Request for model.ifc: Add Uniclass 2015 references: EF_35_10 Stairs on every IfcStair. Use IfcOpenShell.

First a look at what the model holds.

```python
import ifcopenshell

model = ifcopenshell.open("model.ifc")
print(model.schema)
print("classifications:", [c.Name for c in model.by_type("IfcClassification")])
for ifc_class in ("IfcDoor", "IfcRoof", "IfcStair", "IfcWall", "IfcWindow"):
    print(ifc_class, len(model.by_type(ifc_class)))
```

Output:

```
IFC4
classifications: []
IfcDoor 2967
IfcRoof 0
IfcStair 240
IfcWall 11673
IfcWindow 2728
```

```python
import ifcopenshell
import ifcopenshell.api.classification

model = ifcopenshell.open("model.ifc")

system = ifcopenshell.api.classification.add_classification(model, classification="Uniclass 2015")

codes = {
    "IfcStair": ("EF_35_10", "Stairs"),
}
for ifc_class, (code, name) in codes.items():
    products = model.by_type(ifc_class)
    ifcopenshell.api.classification.add_reference(
        model, products=products, classification=system, identification=code, name=name
    )
    print(code, len(products))

model.write("model-out.ifc")
```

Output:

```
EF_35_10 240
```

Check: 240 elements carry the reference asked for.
